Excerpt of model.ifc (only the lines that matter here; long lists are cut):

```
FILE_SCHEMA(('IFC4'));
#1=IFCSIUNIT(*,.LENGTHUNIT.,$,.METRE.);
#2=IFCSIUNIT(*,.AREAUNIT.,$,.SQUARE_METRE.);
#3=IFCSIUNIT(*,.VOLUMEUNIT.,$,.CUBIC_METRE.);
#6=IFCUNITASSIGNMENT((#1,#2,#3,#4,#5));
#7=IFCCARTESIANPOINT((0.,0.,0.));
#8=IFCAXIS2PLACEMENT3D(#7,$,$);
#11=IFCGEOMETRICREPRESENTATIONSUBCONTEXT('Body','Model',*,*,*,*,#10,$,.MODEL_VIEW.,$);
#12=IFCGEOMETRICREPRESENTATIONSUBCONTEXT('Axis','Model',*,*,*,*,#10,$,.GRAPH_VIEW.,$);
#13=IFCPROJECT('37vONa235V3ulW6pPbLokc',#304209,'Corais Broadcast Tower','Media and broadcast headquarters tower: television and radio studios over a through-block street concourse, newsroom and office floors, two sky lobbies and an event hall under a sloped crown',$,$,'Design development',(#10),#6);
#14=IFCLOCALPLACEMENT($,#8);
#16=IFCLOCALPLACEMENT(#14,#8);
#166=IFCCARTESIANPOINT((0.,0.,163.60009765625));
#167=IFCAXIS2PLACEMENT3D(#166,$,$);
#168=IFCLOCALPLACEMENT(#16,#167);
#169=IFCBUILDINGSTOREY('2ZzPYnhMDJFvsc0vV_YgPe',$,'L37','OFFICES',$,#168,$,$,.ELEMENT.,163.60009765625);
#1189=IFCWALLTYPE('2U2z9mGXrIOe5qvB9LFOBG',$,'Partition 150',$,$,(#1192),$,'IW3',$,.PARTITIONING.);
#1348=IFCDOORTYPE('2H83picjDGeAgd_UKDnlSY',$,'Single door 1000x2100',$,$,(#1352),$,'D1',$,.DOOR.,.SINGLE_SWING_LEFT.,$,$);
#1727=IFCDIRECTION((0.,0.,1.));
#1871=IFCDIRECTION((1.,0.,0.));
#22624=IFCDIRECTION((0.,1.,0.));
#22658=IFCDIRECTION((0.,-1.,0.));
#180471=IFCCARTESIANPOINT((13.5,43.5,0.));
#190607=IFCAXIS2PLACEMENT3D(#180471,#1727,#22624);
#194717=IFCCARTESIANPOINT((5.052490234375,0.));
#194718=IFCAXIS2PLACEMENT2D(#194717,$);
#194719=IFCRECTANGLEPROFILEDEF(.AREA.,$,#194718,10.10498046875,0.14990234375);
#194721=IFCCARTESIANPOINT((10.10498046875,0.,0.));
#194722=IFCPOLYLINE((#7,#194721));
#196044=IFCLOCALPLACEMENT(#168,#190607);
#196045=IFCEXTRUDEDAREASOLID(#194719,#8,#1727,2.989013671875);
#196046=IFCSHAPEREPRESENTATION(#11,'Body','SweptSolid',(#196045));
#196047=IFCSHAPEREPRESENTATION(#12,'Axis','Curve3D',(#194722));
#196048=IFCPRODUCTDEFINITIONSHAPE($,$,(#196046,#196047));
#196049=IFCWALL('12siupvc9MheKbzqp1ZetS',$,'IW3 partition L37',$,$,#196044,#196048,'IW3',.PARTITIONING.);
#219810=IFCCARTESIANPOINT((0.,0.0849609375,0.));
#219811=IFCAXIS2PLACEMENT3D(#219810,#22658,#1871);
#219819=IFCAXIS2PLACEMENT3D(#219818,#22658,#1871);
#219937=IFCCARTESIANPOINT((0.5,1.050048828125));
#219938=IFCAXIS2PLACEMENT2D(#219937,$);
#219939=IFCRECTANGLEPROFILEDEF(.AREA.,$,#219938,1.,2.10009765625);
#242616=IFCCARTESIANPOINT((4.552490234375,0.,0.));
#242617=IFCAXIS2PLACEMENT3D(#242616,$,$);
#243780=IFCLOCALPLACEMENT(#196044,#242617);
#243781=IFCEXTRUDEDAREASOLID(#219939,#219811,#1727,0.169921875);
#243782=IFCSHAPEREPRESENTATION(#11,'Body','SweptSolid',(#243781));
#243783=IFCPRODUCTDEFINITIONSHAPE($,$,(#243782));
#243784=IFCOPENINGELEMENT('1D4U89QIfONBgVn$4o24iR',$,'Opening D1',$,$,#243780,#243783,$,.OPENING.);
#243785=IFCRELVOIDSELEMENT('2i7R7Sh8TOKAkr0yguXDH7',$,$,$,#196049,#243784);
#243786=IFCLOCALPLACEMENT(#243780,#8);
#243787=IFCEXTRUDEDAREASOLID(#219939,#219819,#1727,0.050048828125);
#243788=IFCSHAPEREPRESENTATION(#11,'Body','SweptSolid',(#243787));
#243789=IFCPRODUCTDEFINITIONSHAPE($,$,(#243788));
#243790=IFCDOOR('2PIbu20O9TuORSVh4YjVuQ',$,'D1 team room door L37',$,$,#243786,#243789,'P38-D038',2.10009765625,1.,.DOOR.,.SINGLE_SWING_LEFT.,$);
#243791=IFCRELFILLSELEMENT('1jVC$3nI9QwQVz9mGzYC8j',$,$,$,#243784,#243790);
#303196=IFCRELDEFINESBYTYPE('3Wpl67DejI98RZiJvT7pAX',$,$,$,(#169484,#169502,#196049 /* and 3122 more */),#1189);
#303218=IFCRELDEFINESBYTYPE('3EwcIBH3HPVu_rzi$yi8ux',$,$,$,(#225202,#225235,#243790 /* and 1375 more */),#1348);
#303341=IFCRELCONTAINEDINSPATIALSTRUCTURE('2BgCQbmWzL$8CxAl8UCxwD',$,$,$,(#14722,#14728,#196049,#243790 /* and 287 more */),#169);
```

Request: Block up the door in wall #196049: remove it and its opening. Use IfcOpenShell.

```python
import ifcopenshell
import ifcopenshell.api.feature
import ifcopenshell.api.root
import ifcopenshell.geom
import ifcopenshell.util.shape

model = ifcopenshell.open("model.ifc")
settings = ifcopenshell.geom.settings()


def volume(element):
    """Net volume in cubic metres, openings subtracted."""
    shape = ifcopenshell.geom.create_shape(settings, element)
    return ifcopenshell.util.shape.get_volume(shape.geometry)


door = model.by_id(243790)
opening = door.FillsVoids[0].RelatingOpeningElement
wall = opening.VoidsElements[0].RelatingBuildingElement
before = volume(wall)

ifcopenshell.api.root.remove_product(model, product=door)
ifcopenshell.api.feature.remove_feature(model, feature=opening)

after = volume(wall)

print(f"wall volume {before:.3f} -> {after:.3f} m3")

model.write("model-out.ifc")
```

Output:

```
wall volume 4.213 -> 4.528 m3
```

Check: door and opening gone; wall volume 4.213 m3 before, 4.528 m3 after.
